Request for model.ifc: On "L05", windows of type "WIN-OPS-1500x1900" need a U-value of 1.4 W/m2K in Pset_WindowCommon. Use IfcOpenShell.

First a look at what the model holds.

```python
import ifcopenshell
import ifcopenshell.util.element

model = ifcopenshell.open("model.ifc")
print(model.schema)
storey = next(s for s in model.by_type("IfcBuildingStorey") if s.Name == "L05")
windows = [e for e in ifcopenshell.util.element.get_decomposition(storey) if e.is_a("IfcWindow")]
seen = {}
for e in windows:
    element_type = ifcopenshell.util.element.get_type(e)
    key = (element_type.Name if element_type != e and element_type else None, ifcopenshell.util.element.get_pset(e, "Pset_WindowCommon", "ThermalTransmittance"))
    seen[key] = seen.get(key, 0) + 1
for (name, value), count in sorted(seen.items(), key=str):
    print(count, "x", name, "|", value)
```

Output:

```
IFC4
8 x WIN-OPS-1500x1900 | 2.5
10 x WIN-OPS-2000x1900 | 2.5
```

```python
import ifcopenshell
import ifcopenshell.api.pset
import ifcopenshell.util.element

model = ifcopenshell.open("model.ifc")

storey = next(s for s in model.by_type("IfcBuildingStorey") if s.Name == "L05")
windows = [e for e in ifcopenshell.util.element.get_decomposition(storey) if e.is_a("IfcWindow")]

count = 0
for e in windows:
    element_type = ifcopenshell.util.element.get_type(e)
    if element_type in (None, e) or element_type.Name != "WIN-OPS-1500x1900":
        continue
    # add_pset returns the element's existing set when there is one.
    pset = ifcopenshell.api.pset.add_pset(model, product=e, name="Pset_WindowCommon")
    ifcopenshell.api.pset.edit_pset(model, pset=pset, properties={"ThermalTransmittance": 1.4})
    count += 1

print(count, "windows updated")

model.write("model_edited.ifc")
```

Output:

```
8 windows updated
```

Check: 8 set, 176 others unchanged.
